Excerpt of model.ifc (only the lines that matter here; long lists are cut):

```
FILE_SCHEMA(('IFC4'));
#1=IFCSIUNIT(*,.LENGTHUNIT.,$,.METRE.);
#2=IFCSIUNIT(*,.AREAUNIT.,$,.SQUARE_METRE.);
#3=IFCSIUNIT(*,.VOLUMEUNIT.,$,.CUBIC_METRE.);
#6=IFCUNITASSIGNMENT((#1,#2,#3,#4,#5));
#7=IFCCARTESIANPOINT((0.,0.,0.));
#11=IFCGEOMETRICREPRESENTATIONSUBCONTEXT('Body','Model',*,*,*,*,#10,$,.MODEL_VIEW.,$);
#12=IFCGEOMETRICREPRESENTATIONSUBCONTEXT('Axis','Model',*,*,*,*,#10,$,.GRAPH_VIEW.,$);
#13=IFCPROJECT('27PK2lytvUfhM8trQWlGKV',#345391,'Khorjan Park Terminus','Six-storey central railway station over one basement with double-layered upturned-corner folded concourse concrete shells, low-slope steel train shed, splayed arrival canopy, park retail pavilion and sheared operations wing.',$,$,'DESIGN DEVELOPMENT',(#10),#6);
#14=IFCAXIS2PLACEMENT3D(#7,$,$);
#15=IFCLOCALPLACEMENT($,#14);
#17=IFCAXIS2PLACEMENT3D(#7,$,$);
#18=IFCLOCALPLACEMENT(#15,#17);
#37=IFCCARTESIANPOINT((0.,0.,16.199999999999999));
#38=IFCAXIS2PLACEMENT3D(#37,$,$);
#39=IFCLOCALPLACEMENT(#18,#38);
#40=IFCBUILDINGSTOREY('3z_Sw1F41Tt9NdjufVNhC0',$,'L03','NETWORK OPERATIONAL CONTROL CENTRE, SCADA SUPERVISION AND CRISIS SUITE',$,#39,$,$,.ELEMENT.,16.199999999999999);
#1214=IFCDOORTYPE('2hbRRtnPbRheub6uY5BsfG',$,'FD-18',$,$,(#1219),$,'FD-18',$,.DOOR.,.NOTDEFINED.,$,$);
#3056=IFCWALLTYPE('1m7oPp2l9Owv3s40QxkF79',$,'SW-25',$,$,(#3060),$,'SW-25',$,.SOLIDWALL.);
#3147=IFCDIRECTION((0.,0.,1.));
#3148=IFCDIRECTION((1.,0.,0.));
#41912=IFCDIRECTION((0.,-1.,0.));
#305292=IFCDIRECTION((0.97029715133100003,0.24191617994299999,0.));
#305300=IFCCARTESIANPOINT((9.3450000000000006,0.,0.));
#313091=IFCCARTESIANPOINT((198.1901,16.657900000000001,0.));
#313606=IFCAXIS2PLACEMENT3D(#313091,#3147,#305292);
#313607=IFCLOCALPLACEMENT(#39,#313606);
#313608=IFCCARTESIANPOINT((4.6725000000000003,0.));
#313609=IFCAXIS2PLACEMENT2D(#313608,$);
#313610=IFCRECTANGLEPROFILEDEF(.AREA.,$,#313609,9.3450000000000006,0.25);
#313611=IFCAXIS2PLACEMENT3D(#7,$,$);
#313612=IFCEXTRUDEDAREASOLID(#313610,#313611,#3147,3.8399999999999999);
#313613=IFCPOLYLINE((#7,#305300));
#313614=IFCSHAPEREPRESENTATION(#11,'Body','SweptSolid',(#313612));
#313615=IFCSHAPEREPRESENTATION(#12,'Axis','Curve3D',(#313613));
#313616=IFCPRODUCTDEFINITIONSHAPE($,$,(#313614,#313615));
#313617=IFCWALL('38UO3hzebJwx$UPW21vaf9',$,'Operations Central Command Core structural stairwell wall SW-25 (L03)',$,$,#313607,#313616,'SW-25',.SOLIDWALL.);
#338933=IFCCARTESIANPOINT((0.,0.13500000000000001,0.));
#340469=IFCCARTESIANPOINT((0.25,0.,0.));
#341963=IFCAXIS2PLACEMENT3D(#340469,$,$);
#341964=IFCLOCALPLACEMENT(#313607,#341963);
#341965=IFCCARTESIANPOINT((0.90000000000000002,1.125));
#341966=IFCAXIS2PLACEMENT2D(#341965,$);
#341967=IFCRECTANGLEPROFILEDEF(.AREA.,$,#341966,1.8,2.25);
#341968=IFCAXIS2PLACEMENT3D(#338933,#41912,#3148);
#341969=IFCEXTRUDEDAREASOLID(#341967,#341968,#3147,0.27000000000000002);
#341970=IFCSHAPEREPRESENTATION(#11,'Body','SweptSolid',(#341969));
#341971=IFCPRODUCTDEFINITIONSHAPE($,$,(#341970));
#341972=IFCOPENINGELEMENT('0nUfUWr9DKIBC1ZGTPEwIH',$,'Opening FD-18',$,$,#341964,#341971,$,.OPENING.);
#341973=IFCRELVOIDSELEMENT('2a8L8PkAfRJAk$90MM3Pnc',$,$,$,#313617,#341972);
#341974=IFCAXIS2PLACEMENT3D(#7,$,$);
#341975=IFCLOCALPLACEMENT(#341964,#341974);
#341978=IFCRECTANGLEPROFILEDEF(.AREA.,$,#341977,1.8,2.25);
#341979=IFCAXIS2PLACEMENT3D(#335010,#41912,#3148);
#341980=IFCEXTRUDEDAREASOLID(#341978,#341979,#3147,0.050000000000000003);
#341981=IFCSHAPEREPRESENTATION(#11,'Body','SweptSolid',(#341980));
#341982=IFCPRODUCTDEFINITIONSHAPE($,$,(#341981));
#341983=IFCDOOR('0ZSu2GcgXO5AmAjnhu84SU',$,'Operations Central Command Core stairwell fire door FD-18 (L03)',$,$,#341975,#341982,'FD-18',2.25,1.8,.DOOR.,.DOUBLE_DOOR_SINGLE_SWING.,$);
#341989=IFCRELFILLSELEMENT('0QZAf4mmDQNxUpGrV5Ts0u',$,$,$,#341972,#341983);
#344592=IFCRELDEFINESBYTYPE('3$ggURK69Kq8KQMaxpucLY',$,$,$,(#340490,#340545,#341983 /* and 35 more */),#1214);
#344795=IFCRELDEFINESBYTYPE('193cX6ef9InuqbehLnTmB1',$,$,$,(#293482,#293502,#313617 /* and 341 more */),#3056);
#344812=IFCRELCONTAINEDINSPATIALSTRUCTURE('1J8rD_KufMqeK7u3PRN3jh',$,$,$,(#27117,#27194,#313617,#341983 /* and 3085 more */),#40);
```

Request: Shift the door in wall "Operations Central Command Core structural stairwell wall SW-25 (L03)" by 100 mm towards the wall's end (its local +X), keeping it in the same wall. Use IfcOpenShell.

```python
import ifcopenshell
import ifcopenshell.api.geometry
import ifcopenshell.util.placement
import ifcopenshell.util.unit

model = ifcopenshell.open("model.ifc")
unit_scale = ifcopenshell.util.unit.calculate_unit_scale(model)

door = model.by_guid("0ZSu2GcgXO5AmAjnhu84SU")
opening = door.FillsVoids[0].RelatingOpeningElement
wall = opening.VoidsElements[0].RelatingBuildingElement

wall_matrix = ifcopenshell.util.placement.get_local_placement(wall.ObjectPlacement)
shift = wall_matrix[:3, 0] * 0.1 / unit_scale
before = ifcopenshell.util.placement.get_local_placement(door.ObjectPlacement)[:3, 3].copy()

# The door is placed relative to its opening, so it follows when the opening moves.
matrix = ifcopenshell.util.placement.get_local_placement(opening.ObjectPlacement)
matrix[:3, 3] += shift
ifcopenshell.api.geometry.edit_object_placement(
    model, product=opening, matrix=matrix, is_si=False, should_transform_children=True
)

after = ifcopenshell.util.placement.get_local_placement(door.ObjectPlacement)[:3, 3]
print("door moved by", (after - before).round(3) + 0.0)

model.write("model_v2.ifc")
```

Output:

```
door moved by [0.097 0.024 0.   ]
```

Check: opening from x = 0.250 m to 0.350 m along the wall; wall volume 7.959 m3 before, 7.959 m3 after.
